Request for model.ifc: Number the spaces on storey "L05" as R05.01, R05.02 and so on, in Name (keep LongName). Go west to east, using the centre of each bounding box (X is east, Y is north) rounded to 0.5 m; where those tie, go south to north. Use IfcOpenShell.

First a look at what the model holds.

```python
import ifcopenshell
import ifcopenshell.util.element
import ifcopenshell.util.placement

model = ifcopenshell.open("model.ifc")
print(model.schema)
storey = next(s for s in model.by_type("IfcBuildingStorey") if s.Name == "L05")
spaces = [e for e in ifcopenshell.util.element.get_decomposition(storey) if e.is_a("IfcSpace")]
for e in sorted(spaces, key=lambda e: e.id()):
    origin = ifcopenshell.util.placement.get_local_placement(e.ObjectPlacement)[:3, 3]
    print(e.id(), e.Name, e.LongName, origin.round(2) + 0.0, sep=" | ")
```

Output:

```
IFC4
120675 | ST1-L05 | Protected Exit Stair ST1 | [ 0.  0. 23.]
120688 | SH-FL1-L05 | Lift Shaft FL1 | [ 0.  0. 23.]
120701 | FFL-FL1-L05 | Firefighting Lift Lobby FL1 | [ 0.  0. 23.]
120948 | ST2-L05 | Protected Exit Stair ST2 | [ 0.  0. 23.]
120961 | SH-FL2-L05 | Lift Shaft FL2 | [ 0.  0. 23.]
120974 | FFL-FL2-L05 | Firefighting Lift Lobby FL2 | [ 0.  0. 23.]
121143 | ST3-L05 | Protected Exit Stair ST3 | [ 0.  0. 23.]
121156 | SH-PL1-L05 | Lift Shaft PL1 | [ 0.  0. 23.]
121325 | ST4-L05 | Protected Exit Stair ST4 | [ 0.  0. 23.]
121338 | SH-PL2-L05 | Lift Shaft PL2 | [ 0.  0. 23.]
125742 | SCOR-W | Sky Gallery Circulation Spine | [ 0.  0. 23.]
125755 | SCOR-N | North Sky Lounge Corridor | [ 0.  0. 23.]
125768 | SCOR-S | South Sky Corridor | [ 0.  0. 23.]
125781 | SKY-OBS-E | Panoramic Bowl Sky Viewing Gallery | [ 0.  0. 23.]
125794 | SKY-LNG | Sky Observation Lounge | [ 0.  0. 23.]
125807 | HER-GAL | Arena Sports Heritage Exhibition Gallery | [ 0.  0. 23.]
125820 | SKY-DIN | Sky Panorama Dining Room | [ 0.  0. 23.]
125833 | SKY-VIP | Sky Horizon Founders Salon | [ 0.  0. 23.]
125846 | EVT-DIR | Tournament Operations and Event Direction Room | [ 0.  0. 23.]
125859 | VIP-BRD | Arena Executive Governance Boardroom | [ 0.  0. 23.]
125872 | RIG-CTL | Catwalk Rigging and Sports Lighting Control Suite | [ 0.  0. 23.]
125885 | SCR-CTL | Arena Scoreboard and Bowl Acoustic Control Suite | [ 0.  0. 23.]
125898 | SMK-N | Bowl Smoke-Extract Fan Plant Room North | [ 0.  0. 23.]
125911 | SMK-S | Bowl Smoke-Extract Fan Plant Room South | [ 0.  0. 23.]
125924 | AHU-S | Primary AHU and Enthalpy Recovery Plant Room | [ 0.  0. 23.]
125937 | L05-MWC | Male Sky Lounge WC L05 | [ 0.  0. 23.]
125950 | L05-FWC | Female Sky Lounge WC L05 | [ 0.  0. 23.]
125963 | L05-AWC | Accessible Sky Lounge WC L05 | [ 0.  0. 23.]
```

```python
import ifcopenshell
import ifcopenshell.geom
import ifcopenshell.util.element
import ifcopenshell.util.shape

model = ifcopenshell.open("model.ifc")
settings = ifcopenshell.geom.settings()
settings.set("use-world-coords", True)


def centre(element):
    shape = ifcopenshell.geom.create_shape(settings, element)
    return ifcopenshell.util.shape.get_bbox_centroid(shape.geometry)


storey = next(s for s in model.by_type("IfcBuildingStorey") if s.Name == "L05")
spaces = [e for e in ifcopenshell.util.element.get_decomposition(storey) if e.is_a("IfcSpace")]

# Insertion points can sit at a corner or the storey origin, so sort by the geometry (in metres).
centres = {e: centre(e) for e in spaces}
spaces.sort(key=lambda e: (round(centres[e][0] / 0.5), centres[e][1]))

for i, e in enumerate(spaces, start=1):
    number = f"R05.{i:02d}"
    e.Name = number
    print(e.id(), number)

model.write("model_edited.ifc")
```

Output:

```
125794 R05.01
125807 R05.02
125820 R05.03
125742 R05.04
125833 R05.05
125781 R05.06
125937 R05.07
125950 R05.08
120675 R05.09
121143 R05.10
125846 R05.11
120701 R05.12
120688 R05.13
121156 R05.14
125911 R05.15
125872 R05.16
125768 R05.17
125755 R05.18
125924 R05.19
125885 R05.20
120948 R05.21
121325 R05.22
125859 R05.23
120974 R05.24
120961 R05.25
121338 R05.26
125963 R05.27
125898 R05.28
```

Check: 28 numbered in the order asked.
